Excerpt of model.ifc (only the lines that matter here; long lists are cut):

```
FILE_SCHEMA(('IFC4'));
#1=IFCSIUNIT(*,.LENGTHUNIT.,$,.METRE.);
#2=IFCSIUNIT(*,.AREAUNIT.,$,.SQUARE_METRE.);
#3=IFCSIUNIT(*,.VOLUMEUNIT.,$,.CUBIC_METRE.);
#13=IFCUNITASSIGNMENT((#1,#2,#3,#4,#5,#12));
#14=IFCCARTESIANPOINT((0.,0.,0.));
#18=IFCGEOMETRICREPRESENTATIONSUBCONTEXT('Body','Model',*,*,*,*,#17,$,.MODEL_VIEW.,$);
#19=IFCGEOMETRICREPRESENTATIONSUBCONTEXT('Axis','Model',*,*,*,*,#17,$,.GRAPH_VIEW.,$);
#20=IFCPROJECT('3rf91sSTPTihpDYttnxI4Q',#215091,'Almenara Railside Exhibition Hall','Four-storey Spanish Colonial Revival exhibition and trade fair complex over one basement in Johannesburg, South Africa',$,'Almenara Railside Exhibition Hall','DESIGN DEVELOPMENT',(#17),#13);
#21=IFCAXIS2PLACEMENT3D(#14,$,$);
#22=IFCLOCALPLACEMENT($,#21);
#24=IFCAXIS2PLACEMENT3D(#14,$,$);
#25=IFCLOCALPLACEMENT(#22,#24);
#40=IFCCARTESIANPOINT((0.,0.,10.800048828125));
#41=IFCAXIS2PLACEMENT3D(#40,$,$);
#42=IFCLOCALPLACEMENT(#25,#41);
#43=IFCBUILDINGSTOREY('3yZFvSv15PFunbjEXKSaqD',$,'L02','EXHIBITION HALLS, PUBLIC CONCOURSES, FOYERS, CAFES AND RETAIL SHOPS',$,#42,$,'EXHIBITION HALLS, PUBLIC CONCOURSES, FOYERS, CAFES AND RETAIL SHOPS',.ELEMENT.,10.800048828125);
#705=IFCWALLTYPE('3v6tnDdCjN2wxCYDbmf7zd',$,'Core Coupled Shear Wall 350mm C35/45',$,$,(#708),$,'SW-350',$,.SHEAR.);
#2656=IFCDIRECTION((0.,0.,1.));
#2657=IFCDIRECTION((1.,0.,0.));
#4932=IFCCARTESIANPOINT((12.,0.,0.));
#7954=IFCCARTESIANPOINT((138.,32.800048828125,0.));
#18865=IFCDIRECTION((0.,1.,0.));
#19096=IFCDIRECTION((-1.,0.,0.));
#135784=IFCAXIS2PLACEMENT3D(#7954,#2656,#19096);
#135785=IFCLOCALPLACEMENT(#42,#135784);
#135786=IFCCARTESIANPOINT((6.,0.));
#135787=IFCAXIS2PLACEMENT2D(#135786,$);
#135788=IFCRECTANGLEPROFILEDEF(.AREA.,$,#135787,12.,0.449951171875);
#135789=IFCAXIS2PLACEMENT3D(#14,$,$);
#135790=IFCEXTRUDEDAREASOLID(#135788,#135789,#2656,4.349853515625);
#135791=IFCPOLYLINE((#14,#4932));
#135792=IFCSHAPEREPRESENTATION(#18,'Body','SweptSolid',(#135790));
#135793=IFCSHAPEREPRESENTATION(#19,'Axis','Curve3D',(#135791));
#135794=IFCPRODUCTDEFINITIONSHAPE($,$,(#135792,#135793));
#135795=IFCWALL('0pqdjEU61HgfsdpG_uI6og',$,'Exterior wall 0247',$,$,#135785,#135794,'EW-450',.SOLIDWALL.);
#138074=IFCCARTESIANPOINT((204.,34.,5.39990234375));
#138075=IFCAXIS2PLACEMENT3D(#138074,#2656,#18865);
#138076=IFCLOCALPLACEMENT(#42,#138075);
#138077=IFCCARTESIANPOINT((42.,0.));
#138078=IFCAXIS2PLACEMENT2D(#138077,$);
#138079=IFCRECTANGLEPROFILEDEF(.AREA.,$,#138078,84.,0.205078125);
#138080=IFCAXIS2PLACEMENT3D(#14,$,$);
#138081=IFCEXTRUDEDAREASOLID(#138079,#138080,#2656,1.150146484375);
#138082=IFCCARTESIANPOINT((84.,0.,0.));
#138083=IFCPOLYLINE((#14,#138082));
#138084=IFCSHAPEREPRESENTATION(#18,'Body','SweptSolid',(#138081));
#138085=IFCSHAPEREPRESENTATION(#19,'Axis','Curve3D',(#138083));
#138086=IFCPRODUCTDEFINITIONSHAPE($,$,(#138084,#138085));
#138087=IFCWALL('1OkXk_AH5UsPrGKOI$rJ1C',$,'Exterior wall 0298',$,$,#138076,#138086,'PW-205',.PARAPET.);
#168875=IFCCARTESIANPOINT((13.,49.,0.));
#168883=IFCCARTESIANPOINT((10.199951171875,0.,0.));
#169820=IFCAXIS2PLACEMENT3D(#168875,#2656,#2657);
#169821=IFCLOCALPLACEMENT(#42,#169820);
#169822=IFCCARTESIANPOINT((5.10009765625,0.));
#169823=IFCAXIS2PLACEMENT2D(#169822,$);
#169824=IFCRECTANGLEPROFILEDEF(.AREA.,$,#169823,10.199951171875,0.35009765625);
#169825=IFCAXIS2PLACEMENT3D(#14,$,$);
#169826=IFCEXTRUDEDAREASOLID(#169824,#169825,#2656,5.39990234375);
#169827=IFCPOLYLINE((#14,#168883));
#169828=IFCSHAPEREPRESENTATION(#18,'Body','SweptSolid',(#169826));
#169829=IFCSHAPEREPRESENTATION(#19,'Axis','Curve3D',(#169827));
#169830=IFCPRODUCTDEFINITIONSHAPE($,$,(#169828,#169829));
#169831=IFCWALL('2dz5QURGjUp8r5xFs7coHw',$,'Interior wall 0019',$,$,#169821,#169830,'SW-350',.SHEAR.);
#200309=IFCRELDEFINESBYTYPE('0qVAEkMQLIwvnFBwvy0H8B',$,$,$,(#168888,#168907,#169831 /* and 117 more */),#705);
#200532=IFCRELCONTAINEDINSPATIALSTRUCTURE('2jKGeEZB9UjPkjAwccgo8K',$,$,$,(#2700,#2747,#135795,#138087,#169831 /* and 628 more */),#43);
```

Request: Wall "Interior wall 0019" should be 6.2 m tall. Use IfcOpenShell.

```python
import ifcopenshell
import ifcopenshell.geom
import ifcopenshell.util.representation
import ifcopenshell.util.shape
import ifcopenshell.util.unit

model = ifcopenshell.open("model.ifc")
unit_scale = ifcopenshell.util.unit.calculate_unit_scale(model)
settings = ifcopenshell.geom.settings()


def volume(element):
    """Net volume in cubic metres, openings subtracted."""
    shape = ifcopenshell.geom.create_shape(settings, element)
    return ifcopenshell.util.shape.get_volume(shape.geometry)


wall = model.by_guid("2dz5QURGjUp8r5xFs7coHw")
before = volume(wall)

body = ifcopenshell.util.representation.get_representation(wall, "Model", "Body")
solid = body.Items[0]
old_height = solid.Depth
solid.Depth = 6.2 / unit_scale
after = volume(wall)

print(f"height {old_height:g} -> {solid.Depth:g}, volume {before:.3f} -> {after:.3f} m3")

model.write("model_updated.ifc")
```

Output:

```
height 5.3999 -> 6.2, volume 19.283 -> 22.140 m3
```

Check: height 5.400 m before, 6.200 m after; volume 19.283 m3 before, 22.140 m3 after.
